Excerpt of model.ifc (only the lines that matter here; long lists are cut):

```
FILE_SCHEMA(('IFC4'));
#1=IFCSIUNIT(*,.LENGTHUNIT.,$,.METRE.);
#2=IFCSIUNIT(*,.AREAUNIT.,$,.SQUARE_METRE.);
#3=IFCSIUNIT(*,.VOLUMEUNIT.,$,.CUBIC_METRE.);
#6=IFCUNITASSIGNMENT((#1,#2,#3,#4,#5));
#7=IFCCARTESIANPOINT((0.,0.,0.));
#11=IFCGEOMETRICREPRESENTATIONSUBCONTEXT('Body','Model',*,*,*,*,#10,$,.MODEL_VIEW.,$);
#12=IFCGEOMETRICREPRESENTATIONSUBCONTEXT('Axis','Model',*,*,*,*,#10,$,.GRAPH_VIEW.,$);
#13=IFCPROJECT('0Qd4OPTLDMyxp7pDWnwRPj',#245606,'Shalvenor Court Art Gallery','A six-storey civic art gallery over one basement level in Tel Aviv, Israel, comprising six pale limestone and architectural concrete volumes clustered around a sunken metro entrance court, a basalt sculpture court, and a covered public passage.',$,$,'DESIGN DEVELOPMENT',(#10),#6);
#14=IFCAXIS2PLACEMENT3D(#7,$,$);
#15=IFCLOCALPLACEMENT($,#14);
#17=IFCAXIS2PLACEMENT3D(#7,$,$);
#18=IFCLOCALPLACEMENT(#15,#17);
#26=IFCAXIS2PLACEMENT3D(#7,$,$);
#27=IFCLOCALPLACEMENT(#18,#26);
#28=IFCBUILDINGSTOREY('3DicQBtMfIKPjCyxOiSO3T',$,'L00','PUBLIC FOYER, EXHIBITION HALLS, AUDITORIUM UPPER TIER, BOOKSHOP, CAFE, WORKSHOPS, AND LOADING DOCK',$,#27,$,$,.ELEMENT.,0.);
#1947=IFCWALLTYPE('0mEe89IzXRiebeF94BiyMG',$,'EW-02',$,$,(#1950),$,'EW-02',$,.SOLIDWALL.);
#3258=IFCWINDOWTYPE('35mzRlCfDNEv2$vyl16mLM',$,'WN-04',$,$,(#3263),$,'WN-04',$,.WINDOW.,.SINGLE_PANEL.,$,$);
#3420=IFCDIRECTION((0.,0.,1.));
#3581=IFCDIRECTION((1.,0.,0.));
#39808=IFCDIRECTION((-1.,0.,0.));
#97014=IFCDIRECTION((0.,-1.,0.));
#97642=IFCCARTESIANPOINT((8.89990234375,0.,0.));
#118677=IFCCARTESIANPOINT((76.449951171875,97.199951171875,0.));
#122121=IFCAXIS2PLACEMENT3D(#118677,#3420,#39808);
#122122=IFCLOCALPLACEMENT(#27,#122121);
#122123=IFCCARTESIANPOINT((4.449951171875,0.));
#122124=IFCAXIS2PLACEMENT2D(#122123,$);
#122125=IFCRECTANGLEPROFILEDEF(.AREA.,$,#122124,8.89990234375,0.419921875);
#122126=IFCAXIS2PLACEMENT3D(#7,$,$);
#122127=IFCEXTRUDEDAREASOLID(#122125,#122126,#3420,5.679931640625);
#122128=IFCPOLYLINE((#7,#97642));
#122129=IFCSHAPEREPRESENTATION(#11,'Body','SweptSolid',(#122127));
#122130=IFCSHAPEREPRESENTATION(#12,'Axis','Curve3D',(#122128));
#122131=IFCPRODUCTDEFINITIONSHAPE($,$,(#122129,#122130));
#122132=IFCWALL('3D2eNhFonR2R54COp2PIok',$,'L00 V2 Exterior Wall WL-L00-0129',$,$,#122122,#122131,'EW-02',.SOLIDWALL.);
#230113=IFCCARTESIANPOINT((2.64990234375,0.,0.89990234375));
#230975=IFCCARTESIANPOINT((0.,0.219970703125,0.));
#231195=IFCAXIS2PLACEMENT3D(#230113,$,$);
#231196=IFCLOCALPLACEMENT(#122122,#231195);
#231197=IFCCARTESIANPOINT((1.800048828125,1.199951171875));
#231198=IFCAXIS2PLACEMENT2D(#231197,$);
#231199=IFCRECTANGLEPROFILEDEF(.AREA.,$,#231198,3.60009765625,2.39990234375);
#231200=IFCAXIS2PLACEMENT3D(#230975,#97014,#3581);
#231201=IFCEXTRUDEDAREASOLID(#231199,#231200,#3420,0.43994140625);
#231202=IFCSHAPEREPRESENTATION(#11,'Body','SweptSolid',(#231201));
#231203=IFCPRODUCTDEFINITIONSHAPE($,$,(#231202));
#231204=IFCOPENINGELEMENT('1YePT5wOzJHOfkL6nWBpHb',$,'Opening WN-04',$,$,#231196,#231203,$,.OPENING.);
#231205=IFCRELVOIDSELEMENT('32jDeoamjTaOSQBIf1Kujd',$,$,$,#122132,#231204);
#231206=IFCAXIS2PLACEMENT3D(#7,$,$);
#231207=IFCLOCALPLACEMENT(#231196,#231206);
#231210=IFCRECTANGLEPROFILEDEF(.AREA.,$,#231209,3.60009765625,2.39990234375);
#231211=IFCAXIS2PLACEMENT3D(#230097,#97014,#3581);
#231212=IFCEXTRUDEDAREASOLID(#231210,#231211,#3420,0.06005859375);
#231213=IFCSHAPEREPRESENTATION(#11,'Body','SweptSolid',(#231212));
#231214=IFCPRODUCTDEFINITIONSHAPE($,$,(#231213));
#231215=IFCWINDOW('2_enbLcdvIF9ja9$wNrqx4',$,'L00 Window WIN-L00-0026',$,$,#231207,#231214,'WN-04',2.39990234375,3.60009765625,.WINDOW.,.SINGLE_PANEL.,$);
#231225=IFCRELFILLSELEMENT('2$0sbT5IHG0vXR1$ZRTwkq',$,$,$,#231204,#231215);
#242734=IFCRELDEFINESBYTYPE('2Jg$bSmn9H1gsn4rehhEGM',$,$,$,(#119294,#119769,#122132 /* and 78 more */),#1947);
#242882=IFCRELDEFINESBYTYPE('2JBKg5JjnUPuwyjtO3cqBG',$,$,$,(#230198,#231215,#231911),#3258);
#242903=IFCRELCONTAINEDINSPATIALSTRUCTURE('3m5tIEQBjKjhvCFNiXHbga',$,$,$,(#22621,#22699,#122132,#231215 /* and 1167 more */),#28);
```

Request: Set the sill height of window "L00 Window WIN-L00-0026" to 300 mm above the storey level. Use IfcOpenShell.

```python
import numpy as np
import ifcopenshell
import ifcopenshell.api.geometry
import ifcopenshell.geom
import ifcopenshell.util.element
import ifcopenshell.util.placement
import ifcopenshell.util.shape
import ifcopenshell.util.unit

model = ifcopenshell.open("model.ifc")
unit_scale = ifcopenshell.util.unit.calculate_unit_scale(model)

window = model.by_guid("2_enbLcdvIF9ja9$wNrqx4")
opening = window.FillsVoids[0].RelatingOpeningElement
storey = ifcopenshell.util.element.get_container(window, ifc_class="IfcBuildingStorey")
level = ifcopenshell.util.placement.get_local_placement(storey.ObjectPlacement)[2, 3]

# The opening's origin need not be at the sill, so measure its lowest point.
shape = ifcopenshell.geom.create_shape(ifcopenshell.geom.settings(), opening)
bottom = ifcopenshell.util.shape.get_shape_bottom_elevation(shape, shape.geometry) / unit_scale
dz = level + 0.3 - bottom

shift = np.array([0.0, 0.0, dz])
# The window is placed relative to its opening, so it follows when the opening moves.
matrix = ifcopenshell.util.placement.get_local_placement(opening.ObjectPlacement)
matrix[:3, 3] += shift
ifcopenshell.api.geometry.edit_object_placement(
    model, product=opening, matrix=matrix, is_si=False, should_transform_children=True
)

print(f"moved by {dz * unit_scale:+.3f} m")

model.write("model_updated.ifc")
```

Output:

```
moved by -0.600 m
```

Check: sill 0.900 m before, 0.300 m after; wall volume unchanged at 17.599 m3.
